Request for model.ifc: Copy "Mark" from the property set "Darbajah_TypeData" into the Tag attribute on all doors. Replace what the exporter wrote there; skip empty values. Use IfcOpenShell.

First a look at what the model holds.

```python
import ifcopenshell
import ifcopenshell.util.element

model = ifcopenshell.open("model.ifc")
print(model.schema)
doors = model.by_type("IfcDoor")
print(len(doors), "doors")
for e in doors[:8]:
    source = ifcopenshell.util.element.get_pset(e, "Darbajah_TypeData", "Mark")
    target = e.Tag
    print(e.id(), repr(source), repr(target), sep=" | ")
```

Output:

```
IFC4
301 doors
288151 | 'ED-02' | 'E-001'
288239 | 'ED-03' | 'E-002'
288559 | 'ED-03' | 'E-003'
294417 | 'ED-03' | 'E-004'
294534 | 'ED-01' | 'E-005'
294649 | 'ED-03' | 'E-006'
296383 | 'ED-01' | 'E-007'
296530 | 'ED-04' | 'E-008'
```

```python
import ifcopenshell
import ifcopenshell.util.element

model = ifcopenshell.open("model.ifc")

count = 0
for e in model.by_type("IfcDoor"):
    value = ifcopenshell.util.element.get_pset(e, "Darbajah_TypeData", "Mark")
    current = e.Tag
    if not value or not value.strip() or current == value:
        continue
    e.Tag = value
    count += 1

print(count, "doors updated")

model.write("model-out.ifc")
```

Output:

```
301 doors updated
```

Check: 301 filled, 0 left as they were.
